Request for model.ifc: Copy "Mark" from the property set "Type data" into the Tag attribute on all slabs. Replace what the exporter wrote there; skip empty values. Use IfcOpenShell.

First a look at what the model holds.

```python
import ifcopenshell
import ifcopenshell.util.element

model = ifcopenshell.open("model.ifc")
print(model.schema)
slabs = model.by_type("IfcSlab")
print(len(slabs), "slabs")
for e in slabs[:8]:
    source = ifcopenshell.util.element.get_pset(e, "Type data", "Mark")
    target = e.Tag
    print(e.id(), repr(source), repr(target), sep=" | ")
```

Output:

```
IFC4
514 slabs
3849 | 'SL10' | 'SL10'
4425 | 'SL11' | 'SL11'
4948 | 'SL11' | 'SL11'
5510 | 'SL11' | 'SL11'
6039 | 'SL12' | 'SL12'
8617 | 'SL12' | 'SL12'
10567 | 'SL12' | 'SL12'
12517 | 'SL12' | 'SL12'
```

```python
import ifcopenshell
import ifcopenshell.util.element

model = ifcopenshell.open("model.ifc")

count = 0
for e in model.by_type("IfcSlab"):
    value = ifcopenshell.util.element.get_pset(e, "Type data", "Mark")
    current = e.Tag
    if not value or not value.strip() or current == value:
        continue
    e.Tag = value
    count += 1

print(count, "slabs updated")

model.write("model-out.ifc")
```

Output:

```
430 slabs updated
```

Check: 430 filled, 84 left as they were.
